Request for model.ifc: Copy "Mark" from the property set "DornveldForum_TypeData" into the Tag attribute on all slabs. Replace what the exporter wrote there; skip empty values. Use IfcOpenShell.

First a look at what the model holds.

```python
import ifcopenshell
import ifcopenshell.util.element

model = ifcopenshell.open("model.ifc")
print(model.schema)
slabs = model.by_type("IfcSlab")
print(len(slabs), "slabs")
for e in slabs[:8]:
    source = ifcopenshell.util.element.get_pset(e, "DornveldForum_TypeData", "Mark")
    target = e.Tag
    print(e.id(), repr(source), repr(target), sep=" | ")
```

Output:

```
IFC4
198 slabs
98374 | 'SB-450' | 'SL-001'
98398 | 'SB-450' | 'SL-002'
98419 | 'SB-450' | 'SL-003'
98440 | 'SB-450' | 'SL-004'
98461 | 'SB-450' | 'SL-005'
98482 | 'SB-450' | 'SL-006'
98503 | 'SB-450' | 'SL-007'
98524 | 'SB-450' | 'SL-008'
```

```python
import ifcopenshell
import ifcopenshell.util.element

model = ifcopenshell.open("model.ifc")

count = 0
for e in model.by_type("IfcSlab"):
    value = ifcopenshell.util.element.get_pset(e, "DornveldForum_TypeData", "Mark")
    current = e.Tag
    if not value or not value.strip() or current == value:
        continue
    e.Tag = value
    count += 1

print(count, "slabs updated")

model.write("model_v2.ifc")
```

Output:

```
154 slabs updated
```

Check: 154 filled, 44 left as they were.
